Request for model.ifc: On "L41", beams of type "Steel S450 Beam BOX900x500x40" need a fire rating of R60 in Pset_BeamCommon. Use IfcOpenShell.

First a look at what the model holds.

```python
import ifcopenshell
import ifcopenshell.util.element

model = ifcopenshell.open("model.ifc")
print(model.schema)
storey = next(s for s in model.by_type("IfcBuildingStorey") if s.Name == "L41")
beams = [e for e in ifcopenshell.util.element.get_decomposition(storey) if e.is_a("IfcBeam")]
seen = {}
for e in beams:
    element_type = ifcopenshell.util.element.get_type(e)
    key = (element_type.Name if element_type != e and element_type else None, ifcopenshell.util.element.get_pset(e, "Pset_BeamCommon", "FireRating"))
    seen[key] = seen.get(key, 0) + 1
for (name, value), count in sorted(seen.items(), key=str):
    print(count, "x", name, "|", value)
```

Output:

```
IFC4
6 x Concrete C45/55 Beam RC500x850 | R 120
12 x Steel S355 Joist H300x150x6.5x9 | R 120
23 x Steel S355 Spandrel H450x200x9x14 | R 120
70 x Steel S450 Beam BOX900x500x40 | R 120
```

```python
import ifcopenshell
import ifcopenshell.api.pset
import ifcopenshell.util.element

model = ifcopenshell.open("model.ifc")

storey = next(s for s in model.by_type("IfcBuildingStorey") if s.Name == "L41")
beams = [e for e in ifcopenshell.util.element.get_decomposition(storey) if e.is_a("IfcBeam")]

count = 0
for e in beams:
    element_type = ifcopenshell.util.element.get_type(e)
    if element_type in (None, e) or element_type.Name != "Steel S450 Beam BOX900x500x40":
        continue
    found = ifcopenshell.util.element.get_pset(e, "Pset_BeamCommon", should_inherit=False)
    if found:
        pset = model.by_id(found["id"])
        if len(ifcopenshell.util.element.get_elements_by_pset(pset)) > 1:
            pset = ifcopenshell.api.pset.unshare_pset(model, products=[e], pset=pset)[0]
    else:
        pset = ifcopenshell.api.pset.add_pset(model, product=e, name="Pset_BeamCommon")
    ifcopenshell.api.pset.edit_pset(model, pset=pset, properties={"FireRating": "R60"})
    count += 1

print(count, "beams updated")

model.write("model_v2.ifc")
```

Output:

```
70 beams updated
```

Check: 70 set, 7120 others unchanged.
